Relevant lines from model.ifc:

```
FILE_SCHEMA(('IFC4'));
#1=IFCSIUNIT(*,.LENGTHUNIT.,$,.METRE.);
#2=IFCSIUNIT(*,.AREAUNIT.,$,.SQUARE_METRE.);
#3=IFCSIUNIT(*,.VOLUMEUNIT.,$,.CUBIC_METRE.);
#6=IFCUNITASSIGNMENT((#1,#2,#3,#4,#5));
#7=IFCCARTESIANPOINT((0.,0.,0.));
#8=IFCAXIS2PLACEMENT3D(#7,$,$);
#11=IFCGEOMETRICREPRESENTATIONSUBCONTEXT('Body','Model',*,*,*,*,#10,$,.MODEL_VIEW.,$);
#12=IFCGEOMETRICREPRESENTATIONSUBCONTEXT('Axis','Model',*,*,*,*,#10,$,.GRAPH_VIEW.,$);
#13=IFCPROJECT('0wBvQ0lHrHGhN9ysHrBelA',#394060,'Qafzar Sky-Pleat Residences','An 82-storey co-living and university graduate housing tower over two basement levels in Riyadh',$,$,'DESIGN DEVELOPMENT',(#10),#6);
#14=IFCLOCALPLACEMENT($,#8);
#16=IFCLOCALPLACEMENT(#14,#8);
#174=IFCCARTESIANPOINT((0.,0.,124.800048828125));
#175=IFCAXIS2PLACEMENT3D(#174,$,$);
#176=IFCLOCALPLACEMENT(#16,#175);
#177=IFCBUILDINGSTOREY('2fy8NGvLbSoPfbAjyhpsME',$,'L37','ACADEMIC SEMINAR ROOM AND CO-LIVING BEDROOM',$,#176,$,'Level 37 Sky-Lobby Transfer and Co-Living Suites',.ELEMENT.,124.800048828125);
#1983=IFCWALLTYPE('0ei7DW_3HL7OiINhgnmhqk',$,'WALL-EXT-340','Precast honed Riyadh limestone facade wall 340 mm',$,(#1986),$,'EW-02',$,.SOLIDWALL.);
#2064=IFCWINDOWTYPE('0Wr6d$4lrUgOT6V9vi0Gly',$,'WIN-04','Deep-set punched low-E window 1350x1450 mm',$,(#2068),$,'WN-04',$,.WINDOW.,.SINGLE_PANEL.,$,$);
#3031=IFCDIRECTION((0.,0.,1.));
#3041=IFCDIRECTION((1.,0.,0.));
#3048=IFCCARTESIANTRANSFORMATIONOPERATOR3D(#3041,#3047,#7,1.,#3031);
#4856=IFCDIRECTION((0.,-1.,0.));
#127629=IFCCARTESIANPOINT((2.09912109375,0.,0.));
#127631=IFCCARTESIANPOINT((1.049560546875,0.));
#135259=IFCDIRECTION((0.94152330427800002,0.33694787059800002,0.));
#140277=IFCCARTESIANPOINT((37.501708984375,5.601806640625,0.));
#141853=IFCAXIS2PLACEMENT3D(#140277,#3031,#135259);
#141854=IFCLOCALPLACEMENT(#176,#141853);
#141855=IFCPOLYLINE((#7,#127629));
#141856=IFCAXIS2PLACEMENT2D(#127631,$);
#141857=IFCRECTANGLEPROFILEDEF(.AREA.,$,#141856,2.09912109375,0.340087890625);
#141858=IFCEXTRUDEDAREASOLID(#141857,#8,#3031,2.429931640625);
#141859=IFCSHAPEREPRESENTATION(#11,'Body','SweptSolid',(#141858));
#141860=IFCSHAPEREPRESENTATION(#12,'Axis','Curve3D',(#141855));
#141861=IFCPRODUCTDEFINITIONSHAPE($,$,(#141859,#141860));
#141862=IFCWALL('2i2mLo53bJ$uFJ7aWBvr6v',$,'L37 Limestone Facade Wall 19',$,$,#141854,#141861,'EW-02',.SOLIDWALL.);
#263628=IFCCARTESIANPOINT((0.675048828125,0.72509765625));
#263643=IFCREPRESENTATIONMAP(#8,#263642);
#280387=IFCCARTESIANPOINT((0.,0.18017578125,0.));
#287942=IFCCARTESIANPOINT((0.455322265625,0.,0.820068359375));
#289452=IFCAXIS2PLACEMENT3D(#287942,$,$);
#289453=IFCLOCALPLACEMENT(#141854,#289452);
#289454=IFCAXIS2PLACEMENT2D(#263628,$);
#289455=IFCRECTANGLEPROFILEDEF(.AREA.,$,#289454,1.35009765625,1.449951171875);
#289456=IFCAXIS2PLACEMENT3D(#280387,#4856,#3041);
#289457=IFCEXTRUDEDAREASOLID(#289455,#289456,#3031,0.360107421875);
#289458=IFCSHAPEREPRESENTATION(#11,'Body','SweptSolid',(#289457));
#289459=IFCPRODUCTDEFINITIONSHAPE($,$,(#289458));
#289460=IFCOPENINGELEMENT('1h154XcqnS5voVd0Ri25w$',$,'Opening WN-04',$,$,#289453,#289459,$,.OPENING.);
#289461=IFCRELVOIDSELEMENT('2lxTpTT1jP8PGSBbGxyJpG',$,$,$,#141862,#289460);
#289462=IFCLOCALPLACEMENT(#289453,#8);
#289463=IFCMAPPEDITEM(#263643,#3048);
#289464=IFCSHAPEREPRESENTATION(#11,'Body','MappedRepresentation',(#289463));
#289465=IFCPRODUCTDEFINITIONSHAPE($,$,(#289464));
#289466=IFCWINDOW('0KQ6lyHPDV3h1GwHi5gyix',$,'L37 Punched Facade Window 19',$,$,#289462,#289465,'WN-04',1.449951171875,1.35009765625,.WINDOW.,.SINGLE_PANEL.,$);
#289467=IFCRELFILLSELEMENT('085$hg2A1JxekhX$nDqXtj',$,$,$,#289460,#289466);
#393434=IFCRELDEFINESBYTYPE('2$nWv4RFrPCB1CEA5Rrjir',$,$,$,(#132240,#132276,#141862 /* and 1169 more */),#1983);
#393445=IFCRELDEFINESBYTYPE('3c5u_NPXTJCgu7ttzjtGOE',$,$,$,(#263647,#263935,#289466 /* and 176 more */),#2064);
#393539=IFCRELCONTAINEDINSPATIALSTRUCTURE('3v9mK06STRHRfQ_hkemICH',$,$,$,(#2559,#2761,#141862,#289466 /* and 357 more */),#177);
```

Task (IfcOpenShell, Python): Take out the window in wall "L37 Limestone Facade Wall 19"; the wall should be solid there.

```python
import ifcopenshell
import ifcopenshell.api.feature
import ifcopenshell.api.root
import ifcopenshell.geom
import ifcopenshell.util.shape

model = ifcopenshell.open("model.ifc")
settings = ifcopenshell.geom.settings()


def volume(element):
    """Net volume in cubic metres, openings subtracted."""
    shape = ifcopenshell.geom.create_shape(settings, element)
    return ifcopenshell.util.shape.get_volume(shape.geometry)


window = model.by_guid("0KQ6lyHPDV3h1GwHi5gyix")
opening = window.FillsVoids[0].RelatingOpeningElement
wall = opening.VoidsElements[0].RelatingBuildingElement
before = volume(wall)

ifcopenshell.api.root.remove_product(model, product=window)
ifcopenshell.api.feature.remove_feature(model, feature=opening)

after = volume(wall)

print(f"wall volume {before:.3f} -> {after:.3f} m3")

model.write("model-out.ifc")
```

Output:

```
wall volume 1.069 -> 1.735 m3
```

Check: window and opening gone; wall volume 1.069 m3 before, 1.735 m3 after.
